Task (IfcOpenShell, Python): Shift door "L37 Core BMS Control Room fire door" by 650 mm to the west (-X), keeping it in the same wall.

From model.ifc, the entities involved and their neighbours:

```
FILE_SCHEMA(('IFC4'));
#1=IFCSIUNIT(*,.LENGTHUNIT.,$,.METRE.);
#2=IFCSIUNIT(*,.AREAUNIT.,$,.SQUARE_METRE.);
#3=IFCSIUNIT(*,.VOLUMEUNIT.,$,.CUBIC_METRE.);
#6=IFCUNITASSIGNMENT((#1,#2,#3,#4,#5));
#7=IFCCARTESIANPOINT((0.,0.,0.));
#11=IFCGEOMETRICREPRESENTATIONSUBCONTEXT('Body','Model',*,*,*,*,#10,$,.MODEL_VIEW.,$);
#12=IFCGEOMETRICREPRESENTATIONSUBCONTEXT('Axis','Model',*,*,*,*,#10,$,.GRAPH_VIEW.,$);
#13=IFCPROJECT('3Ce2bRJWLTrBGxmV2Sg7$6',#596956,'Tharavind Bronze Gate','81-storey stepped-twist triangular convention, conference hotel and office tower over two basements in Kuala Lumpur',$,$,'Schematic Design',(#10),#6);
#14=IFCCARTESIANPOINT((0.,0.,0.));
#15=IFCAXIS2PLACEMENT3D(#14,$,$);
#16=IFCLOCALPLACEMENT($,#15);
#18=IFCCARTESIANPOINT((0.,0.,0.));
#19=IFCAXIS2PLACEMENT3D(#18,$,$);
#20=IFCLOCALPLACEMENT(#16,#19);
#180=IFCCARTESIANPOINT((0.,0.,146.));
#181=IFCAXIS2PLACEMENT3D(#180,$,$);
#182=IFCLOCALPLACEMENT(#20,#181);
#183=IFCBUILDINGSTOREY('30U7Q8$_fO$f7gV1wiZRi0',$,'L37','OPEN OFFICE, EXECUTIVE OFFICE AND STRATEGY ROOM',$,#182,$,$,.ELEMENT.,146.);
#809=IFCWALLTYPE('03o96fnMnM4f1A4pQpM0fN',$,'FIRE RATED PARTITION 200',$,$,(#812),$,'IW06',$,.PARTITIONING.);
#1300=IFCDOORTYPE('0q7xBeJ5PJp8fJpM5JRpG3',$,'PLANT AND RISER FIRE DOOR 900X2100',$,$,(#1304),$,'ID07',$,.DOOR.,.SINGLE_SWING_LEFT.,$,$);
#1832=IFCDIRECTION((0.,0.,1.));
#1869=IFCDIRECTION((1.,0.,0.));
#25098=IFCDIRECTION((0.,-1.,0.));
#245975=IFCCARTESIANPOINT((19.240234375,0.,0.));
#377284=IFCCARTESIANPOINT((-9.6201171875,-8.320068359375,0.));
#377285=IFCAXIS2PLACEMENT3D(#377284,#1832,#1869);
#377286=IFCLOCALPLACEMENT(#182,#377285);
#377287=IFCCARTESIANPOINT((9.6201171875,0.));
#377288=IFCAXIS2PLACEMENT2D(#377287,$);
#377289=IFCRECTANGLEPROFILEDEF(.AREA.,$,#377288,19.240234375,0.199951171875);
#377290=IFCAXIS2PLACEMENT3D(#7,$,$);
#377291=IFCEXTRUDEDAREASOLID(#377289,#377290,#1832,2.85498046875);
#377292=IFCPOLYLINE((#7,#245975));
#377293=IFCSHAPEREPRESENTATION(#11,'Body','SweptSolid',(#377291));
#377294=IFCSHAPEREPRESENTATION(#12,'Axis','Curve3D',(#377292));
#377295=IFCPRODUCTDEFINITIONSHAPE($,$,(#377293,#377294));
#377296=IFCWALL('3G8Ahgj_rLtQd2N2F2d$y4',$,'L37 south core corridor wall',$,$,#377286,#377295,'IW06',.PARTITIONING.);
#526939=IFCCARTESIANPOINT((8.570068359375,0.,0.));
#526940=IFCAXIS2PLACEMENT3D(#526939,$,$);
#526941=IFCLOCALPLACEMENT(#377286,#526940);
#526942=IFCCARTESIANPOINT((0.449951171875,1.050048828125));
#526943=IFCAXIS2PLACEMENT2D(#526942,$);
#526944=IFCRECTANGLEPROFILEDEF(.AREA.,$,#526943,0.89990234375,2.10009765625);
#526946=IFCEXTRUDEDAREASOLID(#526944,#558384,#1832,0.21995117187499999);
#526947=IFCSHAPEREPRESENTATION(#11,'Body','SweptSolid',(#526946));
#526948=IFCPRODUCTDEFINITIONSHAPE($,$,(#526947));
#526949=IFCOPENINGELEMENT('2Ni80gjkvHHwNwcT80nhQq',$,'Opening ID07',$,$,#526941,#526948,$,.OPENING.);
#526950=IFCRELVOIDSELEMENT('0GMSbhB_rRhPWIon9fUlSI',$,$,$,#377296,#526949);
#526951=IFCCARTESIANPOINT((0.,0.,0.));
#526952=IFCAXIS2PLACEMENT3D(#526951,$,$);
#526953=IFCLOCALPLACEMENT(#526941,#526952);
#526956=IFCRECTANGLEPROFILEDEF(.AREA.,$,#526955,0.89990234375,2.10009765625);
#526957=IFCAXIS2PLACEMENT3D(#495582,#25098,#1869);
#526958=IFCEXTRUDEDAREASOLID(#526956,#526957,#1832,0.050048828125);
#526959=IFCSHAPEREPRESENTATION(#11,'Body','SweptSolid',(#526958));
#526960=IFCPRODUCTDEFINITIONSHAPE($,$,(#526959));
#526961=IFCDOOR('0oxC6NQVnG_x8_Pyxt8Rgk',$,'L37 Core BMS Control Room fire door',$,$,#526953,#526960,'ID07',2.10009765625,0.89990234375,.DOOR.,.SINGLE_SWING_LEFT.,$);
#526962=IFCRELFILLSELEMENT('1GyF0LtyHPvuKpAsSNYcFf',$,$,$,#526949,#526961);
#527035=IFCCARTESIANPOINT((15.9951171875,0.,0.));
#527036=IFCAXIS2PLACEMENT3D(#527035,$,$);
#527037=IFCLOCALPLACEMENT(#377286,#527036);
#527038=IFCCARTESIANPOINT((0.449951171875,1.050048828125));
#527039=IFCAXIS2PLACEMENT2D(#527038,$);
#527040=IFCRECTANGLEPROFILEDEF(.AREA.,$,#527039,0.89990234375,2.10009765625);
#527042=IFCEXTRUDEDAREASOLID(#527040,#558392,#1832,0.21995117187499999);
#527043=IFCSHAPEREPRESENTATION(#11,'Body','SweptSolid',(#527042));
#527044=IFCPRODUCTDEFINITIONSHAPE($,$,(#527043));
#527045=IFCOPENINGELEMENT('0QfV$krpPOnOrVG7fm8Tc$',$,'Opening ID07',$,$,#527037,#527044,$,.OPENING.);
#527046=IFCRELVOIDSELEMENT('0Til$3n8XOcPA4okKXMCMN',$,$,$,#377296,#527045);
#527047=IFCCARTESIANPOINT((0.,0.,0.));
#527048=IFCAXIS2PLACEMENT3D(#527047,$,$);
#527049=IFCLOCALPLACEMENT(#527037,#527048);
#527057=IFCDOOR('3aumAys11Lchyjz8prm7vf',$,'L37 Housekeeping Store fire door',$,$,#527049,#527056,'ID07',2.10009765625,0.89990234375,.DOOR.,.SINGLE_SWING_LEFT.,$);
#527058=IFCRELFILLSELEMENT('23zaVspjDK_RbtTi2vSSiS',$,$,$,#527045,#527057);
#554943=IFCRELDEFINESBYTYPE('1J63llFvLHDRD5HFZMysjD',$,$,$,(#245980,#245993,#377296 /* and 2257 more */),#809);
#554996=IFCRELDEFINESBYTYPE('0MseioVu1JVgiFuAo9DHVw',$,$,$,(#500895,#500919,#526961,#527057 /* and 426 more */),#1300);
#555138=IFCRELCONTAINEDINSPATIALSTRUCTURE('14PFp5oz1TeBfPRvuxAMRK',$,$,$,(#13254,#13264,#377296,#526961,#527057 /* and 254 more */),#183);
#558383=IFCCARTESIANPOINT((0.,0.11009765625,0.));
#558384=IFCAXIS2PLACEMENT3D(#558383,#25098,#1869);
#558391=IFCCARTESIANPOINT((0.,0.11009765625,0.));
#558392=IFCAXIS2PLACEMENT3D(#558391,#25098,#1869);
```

```python
import ifcopenshell
import ifcopenshell.api.geometry
import ifcopenshell.util.placement

model = ifcopenshell.open("model.ifc")

door = model.by_guid("0oxC6NQVnG_x8_Pyxt8Rgk")
opening = door.FillsVoids[0].RelatingOpeningElement
wall = opening.VoidsElements[0].RelatingBuildingElement

wall_matrix = ifcopenshell.util.placement.get_local_placement(wall.ObjectPlacement)
shift = wall_matrix[:3, 0] * -0.65
before = ifcopenshell.util.placement.get_local_placement(door.ObjectPlacement)[:3, 3].copy()

# The door is placed relative to its opening, so it follows when the opening moves.
matrix = ifcopenshell.util.placement.get_local_placement(opening.ObjectPlacement)
matrix[:3, 3] += shift
ifcopenshell.api.geometry.edit_object_placement(
    model, product=opening, matrix=matrix, is_si=False, should_transform_children=True
)

after = ifcopenshell.util.placement.get_local_placement(door.ObjectPlacement)[:3, 3]
print("door moved by", (after - before).round(3) + 0.0)

model.write("model_rev.ifc")
```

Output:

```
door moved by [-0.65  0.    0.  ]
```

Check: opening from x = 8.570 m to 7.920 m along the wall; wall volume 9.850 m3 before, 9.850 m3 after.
